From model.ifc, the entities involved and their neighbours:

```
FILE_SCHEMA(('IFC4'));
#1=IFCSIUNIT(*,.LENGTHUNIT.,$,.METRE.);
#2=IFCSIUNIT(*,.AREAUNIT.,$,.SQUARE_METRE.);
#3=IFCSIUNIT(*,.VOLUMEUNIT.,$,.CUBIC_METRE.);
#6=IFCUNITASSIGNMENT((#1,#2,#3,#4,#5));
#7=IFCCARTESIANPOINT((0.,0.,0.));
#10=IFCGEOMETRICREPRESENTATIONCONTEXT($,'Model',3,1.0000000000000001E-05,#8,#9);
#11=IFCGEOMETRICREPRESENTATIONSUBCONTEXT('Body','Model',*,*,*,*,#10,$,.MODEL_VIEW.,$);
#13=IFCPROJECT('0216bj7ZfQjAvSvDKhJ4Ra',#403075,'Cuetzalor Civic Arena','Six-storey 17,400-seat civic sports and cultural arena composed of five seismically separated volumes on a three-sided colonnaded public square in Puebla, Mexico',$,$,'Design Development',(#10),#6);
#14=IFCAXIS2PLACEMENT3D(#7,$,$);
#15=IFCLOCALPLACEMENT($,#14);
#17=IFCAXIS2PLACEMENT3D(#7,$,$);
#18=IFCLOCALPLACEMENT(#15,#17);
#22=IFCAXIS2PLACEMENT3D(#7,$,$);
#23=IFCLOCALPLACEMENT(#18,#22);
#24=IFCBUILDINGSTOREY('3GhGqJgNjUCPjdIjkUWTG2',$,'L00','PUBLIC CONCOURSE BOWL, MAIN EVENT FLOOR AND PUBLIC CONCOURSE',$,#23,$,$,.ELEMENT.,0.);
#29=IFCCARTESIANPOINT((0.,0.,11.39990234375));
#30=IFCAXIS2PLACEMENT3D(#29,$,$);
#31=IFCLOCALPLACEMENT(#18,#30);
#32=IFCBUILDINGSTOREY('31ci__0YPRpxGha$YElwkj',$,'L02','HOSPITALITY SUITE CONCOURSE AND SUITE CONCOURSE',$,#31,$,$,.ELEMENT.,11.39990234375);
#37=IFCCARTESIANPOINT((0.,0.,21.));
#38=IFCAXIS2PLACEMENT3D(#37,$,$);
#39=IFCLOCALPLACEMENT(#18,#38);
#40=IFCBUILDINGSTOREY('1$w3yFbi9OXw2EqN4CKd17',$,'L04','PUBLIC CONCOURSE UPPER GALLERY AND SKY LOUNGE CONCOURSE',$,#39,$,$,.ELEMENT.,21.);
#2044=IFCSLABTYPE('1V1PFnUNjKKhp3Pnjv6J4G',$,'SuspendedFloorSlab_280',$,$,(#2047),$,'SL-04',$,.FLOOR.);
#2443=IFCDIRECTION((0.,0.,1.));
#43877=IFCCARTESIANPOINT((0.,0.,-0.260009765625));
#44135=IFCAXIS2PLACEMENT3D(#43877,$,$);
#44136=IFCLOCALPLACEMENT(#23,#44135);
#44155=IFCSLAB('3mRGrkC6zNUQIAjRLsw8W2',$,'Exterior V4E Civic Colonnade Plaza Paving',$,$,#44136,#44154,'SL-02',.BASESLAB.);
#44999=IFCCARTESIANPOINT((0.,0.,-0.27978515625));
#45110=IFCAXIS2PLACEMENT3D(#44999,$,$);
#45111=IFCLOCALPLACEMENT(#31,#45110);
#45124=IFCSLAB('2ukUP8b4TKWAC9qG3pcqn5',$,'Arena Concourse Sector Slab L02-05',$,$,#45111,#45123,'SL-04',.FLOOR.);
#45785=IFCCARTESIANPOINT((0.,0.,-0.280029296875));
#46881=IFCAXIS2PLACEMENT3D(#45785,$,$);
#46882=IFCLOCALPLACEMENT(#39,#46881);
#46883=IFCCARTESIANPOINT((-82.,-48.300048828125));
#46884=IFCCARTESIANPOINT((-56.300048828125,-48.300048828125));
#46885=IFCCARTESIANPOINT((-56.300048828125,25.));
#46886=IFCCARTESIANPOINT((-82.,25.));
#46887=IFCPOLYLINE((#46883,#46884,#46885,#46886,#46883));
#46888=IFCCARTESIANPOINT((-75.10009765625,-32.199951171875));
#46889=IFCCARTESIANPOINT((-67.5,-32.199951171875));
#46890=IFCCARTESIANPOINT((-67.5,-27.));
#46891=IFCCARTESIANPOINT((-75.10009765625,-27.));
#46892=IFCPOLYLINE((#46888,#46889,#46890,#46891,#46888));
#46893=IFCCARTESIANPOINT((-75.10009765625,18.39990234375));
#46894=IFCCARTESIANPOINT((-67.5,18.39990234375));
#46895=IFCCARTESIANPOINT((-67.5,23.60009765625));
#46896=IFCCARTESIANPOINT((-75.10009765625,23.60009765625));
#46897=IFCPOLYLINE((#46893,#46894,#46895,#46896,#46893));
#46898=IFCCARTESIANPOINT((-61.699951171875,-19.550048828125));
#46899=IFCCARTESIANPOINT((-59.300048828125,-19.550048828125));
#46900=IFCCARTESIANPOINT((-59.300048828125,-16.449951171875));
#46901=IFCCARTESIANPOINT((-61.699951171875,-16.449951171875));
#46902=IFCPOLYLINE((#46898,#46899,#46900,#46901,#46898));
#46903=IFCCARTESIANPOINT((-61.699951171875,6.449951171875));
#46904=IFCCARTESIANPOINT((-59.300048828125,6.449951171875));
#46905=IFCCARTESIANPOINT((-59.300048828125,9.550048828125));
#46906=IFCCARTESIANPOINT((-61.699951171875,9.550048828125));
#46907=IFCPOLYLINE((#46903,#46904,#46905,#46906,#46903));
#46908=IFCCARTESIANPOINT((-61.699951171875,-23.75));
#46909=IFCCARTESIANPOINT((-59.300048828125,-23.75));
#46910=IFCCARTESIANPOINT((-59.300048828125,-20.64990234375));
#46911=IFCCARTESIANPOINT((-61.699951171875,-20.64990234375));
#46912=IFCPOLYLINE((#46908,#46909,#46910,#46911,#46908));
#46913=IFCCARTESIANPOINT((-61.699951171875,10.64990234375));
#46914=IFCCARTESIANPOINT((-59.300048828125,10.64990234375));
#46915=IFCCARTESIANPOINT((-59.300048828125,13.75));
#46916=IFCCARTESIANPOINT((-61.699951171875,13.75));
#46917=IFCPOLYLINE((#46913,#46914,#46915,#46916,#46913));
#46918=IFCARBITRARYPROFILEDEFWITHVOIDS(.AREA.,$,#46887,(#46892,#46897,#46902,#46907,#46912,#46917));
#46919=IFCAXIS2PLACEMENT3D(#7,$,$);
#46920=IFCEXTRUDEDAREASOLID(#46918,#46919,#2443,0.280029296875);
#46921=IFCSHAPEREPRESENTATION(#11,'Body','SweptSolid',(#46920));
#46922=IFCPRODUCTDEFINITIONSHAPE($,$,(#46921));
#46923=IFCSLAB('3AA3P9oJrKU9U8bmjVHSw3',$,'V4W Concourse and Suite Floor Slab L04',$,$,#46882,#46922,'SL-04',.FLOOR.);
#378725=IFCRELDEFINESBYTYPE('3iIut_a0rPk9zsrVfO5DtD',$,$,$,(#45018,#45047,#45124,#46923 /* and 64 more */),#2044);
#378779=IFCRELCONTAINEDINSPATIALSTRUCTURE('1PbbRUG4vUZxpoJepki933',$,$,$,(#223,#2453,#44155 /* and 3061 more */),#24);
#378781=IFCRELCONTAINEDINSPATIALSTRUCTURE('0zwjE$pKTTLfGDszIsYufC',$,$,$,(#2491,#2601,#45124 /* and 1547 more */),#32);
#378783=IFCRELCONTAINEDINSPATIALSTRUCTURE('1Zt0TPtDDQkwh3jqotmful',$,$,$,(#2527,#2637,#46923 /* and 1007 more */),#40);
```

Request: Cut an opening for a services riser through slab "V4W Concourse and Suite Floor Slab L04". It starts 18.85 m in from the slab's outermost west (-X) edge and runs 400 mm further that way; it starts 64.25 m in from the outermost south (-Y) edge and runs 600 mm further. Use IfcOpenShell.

```python
import numpy as np
import ifcopenshell
import ifcopenshell.api.feature
import ifcopenshell.api.geometry
import ifcopenshell.api.root
import ifcopenshell.geom
import ifcopenshell.util.placement
import ifcopenshell.util.representation
import ifcopenshell.util.shape
import ifcopenshell.util.unit

model = ifcopenshell.open("model.ifc")
unit_scale = ifcopenshell.util.unit.calculate_unit_scale(model)
settings = ifcopenshell.geom.settings()


def volume(element):
    """Net volume in cubic metres, openings subtracted."""
    shape = ifcopenshell.geom.create_shape(settings, element)
    return ifcopenshell.util.shape.get_volume(shape.geometry)


slab = model.by_guid("3AA3P9oJrKU9U8bmjVHSw3")
before = volume(slab)

# Extent in the slab's own axes, in metres. The edges named are its -X and -Y sides.
slab_shape = ifcopenshell.geom.create_shape(settings, slab)
vertices = ifcopenshell.util.shape.get_vertices(slab_shape.geometry)
x_min, y_min, bottom = vertices.min(axis=0)
top = vertices[:, 2].max()

opening = ifcopenshell.api.root.create_entity(model, ifc_class="IfcOpeningElement", name="Services riser opening", predefined_type="OPENING")
context = ifcopenshell.util.representation.get_context(model, "Model", "Body", "MODEL_VIEW")
width, depth = 0.4, 0.6
outline = [(0.0, 0.0), (width, 0.0), (width, depth), (0.0, depth), (0.0, 0.0)]
# Overshoot both faces by 50 mm so the cut is clean.
shape = ifcopenshell.api.geometry.add_slab_representation(
    model, context=context, depth=top - bottom + 0.1, polyline=outline
)
ifcopenshell.api.geometry.assign_representation(model, product=opening, representation=shape)

matrix = ifcopenshell.util.placement.get_local_placement(slab.ObjectPlacement)
matrix[:, 3] = matrix @ np.append(np.array([x_min + 18.85, y_min + 64.25, bottom - 0.05]) / unit_scale, 1.0)
ifcopenshell.api.geometry.edit_object_placement(model, product=opening, matrix=matrix, is_si=False)
ifcopenshell.api.feature.add_feature(model, feature=opening, element=slab)

after = volume(slab)

print(f"slab volume {before:.3f} -> {after:.3f} m3")

model.write("model_rev.ifc")
```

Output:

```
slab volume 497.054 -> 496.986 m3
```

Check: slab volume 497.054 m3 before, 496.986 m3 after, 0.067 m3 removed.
